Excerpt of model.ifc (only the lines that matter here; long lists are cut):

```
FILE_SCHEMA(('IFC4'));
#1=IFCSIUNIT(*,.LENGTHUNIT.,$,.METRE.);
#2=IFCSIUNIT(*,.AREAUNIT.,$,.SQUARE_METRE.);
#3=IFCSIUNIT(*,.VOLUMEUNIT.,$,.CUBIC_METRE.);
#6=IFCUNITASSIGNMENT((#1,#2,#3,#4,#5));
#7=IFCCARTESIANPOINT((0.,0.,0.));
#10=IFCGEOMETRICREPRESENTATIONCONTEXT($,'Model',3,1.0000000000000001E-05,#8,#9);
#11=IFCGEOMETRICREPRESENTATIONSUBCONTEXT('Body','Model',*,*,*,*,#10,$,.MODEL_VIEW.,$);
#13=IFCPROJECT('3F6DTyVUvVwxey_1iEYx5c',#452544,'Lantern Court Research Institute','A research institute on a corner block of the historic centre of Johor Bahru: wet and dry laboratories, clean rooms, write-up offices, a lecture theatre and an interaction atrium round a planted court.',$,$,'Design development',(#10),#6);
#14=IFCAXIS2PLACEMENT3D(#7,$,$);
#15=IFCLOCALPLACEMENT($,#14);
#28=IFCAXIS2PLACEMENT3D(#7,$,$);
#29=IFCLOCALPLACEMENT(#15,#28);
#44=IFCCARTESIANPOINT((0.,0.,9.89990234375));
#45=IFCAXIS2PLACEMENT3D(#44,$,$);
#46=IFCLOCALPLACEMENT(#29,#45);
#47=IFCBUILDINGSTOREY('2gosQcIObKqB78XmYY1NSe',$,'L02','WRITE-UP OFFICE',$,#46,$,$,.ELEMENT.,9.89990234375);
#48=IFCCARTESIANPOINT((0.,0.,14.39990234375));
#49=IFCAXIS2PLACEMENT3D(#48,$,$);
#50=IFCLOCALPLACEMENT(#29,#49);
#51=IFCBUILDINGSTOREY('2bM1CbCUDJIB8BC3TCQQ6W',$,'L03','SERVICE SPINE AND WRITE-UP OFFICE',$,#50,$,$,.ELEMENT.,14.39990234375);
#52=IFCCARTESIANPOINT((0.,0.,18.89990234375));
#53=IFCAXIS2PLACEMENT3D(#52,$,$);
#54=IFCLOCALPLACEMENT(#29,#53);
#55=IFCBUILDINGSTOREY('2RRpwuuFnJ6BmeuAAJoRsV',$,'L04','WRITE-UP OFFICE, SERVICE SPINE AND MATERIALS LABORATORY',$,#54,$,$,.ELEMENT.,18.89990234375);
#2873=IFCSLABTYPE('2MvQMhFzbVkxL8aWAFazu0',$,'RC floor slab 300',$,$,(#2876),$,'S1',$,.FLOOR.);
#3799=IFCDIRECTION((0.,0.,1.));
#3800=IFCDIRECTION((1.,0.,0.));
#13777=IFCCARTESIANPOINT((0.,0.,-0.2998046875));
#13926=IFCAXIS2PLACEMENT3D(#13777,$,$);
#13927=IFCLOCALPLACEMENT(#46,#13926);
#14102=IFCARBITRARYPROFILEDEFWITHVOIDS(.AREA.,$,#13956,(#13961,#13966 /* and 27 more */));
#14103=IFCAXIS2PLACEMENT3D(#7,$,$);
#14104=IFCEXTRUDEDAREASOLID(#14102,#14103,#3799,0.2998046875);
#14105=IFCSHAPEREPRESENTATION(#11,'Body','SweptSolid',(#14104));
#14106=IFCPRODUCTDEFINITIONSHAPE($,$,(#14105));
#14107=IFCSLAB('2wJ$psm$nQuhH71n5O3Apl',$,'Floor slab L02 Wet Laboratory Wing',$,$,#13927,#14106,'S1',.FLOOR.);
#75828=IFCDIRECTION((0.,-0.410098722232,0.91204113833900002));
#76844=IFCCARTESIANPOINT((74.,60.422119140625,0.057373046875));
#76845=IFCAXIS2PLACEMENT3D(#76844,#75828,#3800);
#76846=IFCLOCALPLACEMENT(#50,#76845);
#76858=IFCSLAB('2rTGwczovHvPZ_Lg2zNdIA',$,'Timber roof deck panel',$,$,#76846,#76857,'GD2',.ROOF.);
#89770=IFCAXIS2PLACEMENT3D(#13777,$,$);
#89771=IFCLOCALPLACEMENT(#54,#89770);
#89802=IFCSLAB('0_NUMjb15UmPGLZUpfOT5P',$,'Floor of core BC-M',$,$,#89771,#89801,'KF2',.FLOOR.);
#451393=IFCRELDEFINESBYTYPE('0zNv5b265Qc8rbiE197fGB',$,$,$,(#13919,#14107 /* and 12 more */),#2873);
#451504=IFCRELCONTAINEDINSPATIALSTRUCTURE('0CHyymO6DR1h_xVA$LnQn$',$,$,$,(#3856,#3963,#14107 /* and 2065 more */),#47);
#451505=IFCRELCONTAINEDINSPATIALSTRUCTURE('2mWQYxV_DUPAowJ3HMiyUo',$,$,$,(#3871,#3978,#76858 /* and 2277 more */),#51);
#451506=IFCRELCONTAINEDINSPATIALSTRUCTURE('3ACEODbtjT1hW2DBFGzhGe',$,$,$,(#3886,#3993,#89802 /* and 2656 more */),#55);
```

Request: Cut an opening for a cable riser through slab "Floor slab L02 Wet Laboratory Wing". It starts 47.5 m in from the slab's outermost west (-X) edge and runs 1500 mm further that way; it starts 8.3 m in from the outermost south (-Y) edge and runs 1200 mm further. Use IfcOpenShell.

```python
import numpy as np
import ifcopenshell
import ifcopenshell.api.feature
import ifcopenshell.api.geometry
import ifcopenshell.api.root
import ifcopenshell.geom
import ifcopenshell.util.placement
import ifcopenshell.util.representation
import ifcopenshell.util.shape
import ifcopenshell.util.unit

model = ifcopenshell.open("model.ifc")
unit_scale = ifcopenshell.util.unit.calculate_unit_scale(model)
settings = ifcopenshell.geom.settings()


def volume(element):
    """Net volume in cubic metres, openings subtracted."""
    shape = ifcopenshell.geom.create_shape(settings, element)
    return ifcopenshell.util.shape.get_volume(shape.geometry)


slab = model.by_id(14107)
before = volume(slab)

# Extent in the slab's own axes, in metres. The edges named are its -X and -Y sides.
slab_shape = ifcopenshell.geom.create_shape(settings, slab)
vertices = ifcopenshell.util.shape.get_vertices(slab_shape.geometry)
x_min, y_min, bottom = vertices.min(axis=0)
top = vertices[:, 2].max()

opening = ifcopenshell.api.root.create_entity(model, ifc_class="IfcOpeningElement", name="Cable riser opening", predefined_type="OPENING")
context = ifcopenshell.util.representation.get_context(model, "Model", "Body", "MODEL_VIEW")
width, depth = 1.5, 1.2
outline = [(0.0, 0.0), (width, 0.0), (width, depth), (0.0, depth), (0.0, 0.0)]
# Overshoot both faces by 50 mm so the cut is clean.
shape = ifcopenshell.api.geometry.add_slab_representation(
    model, context=context, depth=top - bottom + 0.1, polyline=outline
)
ifcopenshell.api.geometry.assign_representation(model, product=opening, representation=shape)

matrix = ifcopenshell.util.placement.get_local_placement(slab.ObjectPlacement)
matrix[:, 3] = matrix @ np.append(np.array([x_min + 47.5, y_min + 8.3, bottom - 0.05]) / unit_scale, 1.0)
ifcopenshell.api.geometry.edit_object_placement(model, product=opening, matrix=matrix, is_si=False)
ifcopenshell.api.feature.add_feature(model, feature=opening, element=slab)

after = volume(slab)

print(f"slab volume {before:.3f} -> {after:.3f} m3")

model.write("model_rev.ifc")
```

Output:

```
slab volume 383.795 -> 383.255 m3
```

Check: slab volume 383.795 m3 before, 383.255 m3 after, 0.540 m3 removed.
